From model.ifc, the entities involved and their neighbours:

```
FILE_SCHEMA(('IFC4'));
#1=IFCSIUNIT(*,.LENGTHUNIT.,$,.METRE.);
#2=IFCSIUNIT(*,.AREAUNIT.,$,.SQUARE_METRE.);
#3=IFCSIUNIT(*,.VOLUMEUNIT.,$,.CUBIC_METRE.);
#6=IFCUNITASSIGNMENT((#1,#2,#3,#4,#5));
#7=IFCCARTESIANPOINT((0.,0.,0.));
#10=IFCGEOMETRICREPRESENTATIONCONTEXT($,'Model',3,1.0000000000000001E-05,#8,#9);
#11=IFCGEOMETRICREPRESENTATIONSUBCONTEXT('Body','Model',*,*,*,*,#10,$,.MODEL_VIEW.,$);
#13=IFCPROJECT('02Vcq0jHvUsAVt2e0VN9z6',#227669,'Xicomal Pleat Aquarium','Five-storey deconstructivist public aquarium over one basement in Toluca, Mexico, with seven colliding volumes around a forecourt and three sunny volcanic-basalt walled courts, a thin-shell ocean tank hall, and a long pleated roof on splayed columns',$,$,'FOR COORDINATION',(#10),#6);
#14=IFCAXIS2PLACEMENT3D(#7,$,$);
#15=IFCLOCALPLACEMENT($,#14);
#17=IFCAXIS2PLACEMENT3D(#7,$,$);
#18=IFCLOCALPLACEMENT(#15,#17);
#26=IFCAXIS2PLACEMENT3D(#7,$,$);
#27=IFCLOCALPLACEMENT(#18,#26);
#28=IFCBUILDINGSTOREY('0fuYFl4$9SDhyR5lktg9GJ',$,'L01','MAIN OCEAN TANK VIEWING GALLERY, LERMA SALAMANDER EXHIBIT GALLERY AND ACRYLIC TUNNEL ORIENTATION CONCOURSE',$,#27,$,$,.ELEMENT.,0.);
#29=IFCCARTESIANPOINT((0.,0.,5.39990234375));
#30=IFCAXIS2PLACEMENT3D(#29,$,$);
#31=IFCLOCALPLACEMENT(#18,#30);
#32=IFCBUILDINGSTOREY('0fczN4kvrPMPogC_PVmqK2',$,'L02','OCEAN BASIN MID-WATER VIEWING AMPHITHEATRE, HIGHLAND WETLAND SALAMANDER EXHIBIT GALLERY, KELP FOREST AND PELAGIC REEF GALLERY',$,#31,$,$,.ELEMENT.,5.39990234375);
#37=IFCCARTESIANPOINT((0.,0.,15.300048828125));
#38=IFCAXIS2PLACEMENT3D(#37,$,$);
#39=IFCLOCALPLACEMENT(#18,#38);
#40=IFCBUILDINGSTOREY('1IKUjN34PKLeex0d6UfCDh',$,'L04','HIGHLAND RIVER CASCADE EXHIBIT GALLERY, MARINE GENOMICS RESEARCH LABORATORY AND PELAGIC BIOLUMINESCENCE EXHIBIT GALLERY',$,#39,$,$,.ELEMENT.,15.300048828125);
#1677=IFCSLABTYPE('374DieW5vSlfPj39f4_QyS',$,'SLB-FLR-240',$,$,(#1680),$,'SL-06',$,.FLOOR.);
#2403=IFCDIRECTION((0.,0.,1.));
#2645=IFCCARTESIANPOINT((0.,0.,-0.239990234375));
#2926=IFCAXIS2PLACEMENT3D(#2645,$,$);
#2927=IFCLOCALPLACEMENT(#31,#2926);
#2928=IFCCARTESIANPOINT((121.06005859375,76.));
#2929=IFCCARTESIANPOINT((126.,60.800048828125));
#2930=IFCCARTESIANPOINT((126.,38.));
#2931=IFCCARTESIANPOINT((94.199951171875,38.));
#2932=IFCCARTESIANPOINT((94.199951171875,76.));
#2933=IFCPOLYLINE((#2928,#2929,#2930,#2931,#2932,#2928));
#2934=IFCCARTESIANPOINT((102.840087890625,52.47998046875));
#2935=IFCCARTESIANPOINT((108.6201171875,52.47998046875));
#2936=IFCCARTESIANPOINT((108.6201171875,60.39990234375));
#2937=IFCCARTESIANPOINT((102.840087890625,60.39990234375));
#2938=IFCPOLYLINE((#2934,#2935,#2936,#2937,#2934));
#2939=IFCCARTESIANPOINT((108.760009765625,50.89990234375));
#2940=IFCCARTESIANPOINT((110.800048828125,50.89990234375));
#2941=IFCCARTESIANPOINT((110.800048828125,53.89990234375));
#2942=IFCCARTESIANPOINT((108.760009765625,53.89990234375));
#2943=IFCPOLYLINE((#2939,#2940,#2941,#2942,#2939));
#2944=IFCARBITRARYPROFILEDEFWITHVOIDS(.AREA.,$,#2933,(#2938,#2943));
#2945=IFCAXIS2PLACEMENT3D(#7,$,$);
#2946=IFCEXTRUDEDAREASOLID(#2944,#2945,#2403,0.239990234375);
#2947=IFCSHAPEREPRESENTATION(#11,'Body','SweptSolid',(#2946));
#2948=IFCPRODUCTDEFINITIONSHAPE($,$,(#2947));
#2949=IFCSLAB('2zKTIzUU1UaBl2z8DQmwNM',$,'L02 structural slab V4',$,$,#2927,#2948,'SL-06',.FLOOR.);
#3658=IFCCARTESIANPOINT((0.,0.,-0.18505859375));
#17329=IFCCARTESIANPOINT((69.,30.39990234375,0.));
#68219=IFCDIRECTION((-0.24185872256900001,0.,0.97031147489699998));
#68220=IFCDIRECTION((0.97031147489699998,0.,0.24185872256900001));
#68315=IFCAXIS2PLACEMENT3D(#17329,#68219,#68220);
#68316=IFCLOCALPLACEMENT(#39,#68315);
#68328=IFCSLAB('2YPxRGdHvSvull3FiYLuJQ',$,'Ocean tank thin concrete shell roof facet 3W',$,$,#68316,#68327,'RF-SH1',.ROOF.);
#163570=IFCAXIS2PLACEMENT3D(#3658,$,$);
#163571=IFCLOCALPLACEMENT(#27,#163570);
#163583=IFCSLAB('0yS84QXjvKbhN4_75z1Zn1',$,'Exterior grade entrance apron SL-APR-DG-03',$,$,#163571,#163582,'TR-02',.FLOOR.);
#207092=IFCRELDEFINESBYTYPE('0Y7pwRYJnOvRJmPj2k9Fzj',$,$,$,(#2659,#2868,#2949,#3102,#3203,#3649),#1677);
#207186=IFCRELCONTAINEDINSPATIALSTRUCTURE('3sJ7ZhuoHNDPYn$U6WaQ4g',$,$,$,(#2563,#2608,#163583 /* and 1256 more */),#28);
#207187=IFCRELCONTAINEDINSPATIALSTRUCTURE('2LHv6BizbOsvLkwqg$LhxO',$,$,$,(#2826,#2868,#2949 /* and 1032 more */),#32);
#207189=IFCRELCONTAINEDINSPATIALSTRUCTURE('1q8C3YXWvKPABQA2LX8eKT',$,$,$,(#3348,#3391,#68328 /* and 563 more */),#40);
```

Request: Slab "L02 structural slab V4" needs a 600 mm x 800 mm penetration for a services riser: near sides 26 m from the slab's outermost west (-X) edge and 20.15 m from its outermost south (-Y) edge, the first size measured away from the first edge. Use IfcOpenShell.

```python
import numpy as np
import ifcopenshell
import ifcopenshell.api.feature
import ifcopenshell.api.geometry
import ifcopenshell.api.root
import ifcopenshell.geom
import ifcopenshell.util.placement
import ifcopenshell.util.representation
import ifcopenshell.util.shape
import ifcopenshell.util.unit

model = ifcopenshell.open("model.ifc")
unit_scale = ifcopenshell.util.unit.calculate_unit_scale(model)
settings = ifcopenshell.geom.settings()


def volume(element):
    """Net volume in cubic metres, openings subtracted."""
    shape = ifcopenshell.geom.create_shape(settings, element)
    return ifcopenshell.util.shape.get_volume(shape.geometry)


slab = model.by_id(2949)
before = volume(slab)

# Extent in the slab's own axes, in metres. The edges named are its -X and -Y sides.
slab_shape = ifcopenshell.geom.create_shape(settings, slab)
vertices = ifcopenshell.util.shape.get_vertices(slab_shape.geometry)
x_min, y_min, bottom = vertices.min(axis=0)
top = vertices[:, 2].max()

opening = ifcopenshell.api.root.create_entity(model, ifc_class="IfcOpeningElement", name="Services riser opening", predefined_type="OPENING")
context = ifcopenshell.util.representation.get_context(model, "Model", "Body", "MODEL_VIEW")
width, depth = 0.6, 0.8
outline = [(0.0, 0.0), (width, 0.0), (width, depth), (0.0, depth), (0.0, 0.0)]
# Overshoot both faces by 50 mm so the cut is clean.
shape = ifcopenshell.api.geometry.add_slab_representation(
    model, context=context, depth=top - bottom + 0.1, polyline=outline
)
ifcopenshell.api.geometry.assign_representation(model, product=opening, representation=shape)

matrix = ifcopenshell.util.placement.get_local_placement(slab.ObjectPlacement)
matrix[:, 3] = matrix @ np.append(np.array([x_min + 26, y_min + 20.15, bottom - 0.05]) / unit_scale, 1.0)
ifcopenshell.api.geometry.edit_object_placement(model, product=opening, matrix=matrix, is_si=False)
ifcopenshell.api.feature.add_feature(model, feature=opening, element=slab)

after = volume(slab)

print(f"slab volume {before:.3f} -> {after:.3f} m3")

model.write("model_v2.ifc")
```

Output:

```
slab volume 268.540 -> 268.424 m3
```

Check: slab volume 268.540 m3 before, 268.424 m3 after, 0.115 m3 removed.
